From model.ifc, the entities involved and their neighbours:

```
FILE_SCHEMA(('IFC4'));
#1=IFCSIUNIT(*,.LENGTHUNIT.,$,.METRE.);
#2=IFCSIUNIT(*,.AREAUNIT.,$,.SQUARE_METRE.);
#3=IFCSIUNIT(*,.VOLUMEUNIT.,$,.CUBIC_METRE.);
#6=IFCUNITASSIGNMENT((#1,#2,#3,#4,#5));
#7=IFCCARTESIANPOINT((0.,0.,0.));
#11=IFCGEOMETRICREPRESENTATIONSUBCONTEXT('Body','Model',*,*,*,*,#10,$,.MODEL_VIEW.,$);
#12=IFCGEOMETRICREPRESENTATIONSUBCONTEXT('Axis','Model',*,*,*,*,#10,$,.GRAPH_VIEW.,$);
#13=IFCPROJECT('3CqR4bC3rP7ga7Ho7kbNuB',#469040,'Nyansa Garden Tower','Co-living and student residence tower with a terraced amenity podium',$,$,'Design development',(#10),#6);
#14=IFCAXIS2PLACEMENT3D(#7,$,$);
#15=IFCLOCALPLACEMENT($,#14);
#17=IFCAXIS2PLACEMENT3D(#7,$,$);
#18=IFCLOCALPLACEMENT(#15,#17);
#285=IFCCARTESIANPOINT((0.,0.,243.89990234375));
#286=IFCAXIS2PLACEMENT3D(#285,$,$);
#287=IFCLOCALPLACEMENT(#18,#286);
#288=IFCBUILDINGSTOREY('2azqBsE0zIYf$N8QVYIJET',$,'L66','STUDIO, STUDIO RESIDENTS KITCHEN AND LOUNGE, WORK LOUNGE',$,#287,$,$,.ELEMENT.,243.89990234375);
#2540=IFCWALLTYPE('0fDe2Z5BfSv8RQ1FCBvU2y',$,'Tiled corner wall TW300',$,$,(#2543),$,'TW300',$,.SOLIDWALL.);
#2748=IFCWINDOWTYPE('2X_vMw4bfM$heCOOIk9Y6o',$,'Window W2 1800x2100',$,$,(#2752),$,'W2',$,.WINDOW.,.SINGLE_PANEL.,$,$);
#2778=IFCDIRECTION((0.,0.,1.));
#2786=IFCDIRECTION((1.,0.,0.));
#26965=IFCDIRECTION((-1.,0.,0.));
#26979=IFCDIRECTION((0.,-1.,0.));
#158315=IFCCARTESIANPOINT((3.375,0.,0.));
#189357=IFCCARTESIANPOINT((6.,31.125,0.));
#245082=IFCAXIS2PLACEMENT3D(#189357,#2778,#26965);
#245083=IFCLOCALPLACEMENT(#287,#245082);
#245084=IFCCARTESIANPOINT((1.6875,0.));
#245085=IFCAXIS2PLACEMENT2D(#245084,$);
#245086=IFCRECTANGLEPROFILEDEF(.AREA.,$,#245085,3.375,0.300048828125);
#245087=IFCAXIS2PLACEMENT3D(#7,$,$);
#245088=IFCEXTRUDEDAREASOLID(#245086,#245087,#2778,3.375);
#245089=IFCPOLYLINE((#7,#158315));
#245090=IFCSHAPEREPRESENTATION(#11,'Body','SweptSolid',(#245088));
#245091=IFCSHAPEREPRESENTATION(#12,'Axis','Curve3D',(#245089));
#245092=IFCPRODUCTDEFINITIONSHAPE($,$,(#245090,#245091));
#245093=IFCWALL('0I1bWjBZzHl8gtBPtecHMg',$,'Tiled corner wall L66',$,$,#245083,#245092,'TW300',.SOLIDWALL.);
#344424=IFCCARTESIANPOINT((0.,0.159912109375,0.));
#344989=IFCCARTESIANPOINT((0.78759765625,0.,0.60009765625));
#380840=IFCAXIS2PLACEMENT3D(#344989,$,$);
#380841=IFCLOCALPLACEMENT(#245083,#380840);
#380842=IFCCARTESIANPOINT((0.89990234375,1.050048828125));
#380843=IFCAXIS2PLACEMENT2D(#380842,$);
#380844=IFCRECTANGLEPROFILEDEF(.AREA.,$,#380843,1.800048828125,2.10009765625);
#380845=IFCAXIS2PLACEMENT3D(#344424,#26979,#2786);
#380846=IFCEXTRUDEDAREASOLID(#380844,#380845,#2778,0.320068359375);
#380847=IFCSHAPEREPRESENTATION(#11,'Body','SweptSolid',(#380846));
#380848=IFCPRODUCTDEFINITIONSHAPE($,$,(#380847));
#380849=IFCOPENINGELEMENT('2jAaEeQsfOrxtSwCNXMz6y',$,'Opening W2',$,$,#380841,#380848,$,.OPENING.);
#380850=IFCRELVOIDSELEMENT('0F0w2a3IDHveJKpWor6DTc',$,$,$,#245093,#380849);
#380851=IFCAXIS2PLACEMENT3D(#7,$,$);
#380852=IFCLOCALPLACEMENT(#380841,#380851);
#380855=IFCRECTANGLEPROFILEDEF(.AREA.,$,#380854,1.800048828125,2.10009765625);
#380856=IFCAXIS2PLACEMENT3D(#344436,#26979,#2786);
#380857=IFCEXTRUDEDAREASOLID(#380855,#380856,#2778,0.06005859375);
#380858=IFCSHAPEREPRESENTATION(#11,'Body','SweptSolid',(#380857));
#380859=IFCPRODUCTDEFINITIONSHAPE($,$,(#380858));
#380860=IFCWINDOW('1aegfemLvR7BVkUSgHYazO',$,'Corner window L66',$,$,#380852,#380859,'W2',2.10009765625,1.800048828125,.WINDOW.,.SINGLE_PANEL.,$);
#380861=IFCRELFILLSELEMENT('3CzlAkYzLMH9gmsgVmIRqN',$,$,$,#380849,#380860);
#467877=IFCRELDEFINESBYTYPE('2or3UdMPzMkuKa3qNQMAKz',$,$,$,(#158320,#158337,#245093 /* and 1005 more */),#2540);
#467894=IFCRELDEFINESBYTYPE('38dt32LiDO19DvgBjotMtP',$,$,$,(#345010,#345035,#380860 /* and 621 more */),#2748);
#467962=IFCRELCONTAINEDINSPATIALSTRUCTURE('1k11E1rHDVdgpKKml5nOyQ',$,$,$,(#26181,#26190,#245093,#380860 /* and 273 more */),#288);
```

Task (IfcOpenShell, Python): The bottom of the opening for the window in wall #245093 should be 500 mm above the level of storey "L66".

```python
import numpy as np
import ifcopenshell
import ifcopenshell.api.geometry
import ifcopenshell.geom
import ifcopenshell.util.element
import ifcopenshell.util.placement
import ifcopenshell.util.shape
import ifcopenshell.util.unit

model = ifcopenshell.open("model.ifc")
unit_scale = ifcopenshell.util.unit.calculate_unit_scale(model)

window = model.by_guid("1aegfemLvR7BVkUSgHYazO")
opening = window.FillsVoids[0].RelatingOpeningElement
storey = ifcopenshell.util.element.get_container(window, ifc_class="IfcBuildingStorey")
level = ifcopenshell.util.placement.get_local_placement(storey.ObjectPlacement)[2, 3]

# The opening's origin need not be at the sill, so measure its lowest point.
shape = ifcopenshell.geom.create_shape(ifcopenshell.geom.settings(), opening)
bottom = ifcopenshell.util.shape.get_shape_bottom_elevation(shape, shape.geometry) / unit_scale
dz = level + 0.5 / unit_scale - bottom

shift = np.array([0.0, 0.0, dz])
# The window is placed relative to its opening, so it follows when the opening moves.
matrix = ifcopenshell.util.placement.get_local_placement(opening.ObjectPlacement)
matrix[:3, 3] += shift
ifcopenshell.api.geometry.edit_object_placement(
    model, product=opening, matrix=matrix, is_si=False, should_transform_children=True
)

print(f"moved by {dz * unit_scale:+.3f} m")

model.write("model_edited.ifc")
```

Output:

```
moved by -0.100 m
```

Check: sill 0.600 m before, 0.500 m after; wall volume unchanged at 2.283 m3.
